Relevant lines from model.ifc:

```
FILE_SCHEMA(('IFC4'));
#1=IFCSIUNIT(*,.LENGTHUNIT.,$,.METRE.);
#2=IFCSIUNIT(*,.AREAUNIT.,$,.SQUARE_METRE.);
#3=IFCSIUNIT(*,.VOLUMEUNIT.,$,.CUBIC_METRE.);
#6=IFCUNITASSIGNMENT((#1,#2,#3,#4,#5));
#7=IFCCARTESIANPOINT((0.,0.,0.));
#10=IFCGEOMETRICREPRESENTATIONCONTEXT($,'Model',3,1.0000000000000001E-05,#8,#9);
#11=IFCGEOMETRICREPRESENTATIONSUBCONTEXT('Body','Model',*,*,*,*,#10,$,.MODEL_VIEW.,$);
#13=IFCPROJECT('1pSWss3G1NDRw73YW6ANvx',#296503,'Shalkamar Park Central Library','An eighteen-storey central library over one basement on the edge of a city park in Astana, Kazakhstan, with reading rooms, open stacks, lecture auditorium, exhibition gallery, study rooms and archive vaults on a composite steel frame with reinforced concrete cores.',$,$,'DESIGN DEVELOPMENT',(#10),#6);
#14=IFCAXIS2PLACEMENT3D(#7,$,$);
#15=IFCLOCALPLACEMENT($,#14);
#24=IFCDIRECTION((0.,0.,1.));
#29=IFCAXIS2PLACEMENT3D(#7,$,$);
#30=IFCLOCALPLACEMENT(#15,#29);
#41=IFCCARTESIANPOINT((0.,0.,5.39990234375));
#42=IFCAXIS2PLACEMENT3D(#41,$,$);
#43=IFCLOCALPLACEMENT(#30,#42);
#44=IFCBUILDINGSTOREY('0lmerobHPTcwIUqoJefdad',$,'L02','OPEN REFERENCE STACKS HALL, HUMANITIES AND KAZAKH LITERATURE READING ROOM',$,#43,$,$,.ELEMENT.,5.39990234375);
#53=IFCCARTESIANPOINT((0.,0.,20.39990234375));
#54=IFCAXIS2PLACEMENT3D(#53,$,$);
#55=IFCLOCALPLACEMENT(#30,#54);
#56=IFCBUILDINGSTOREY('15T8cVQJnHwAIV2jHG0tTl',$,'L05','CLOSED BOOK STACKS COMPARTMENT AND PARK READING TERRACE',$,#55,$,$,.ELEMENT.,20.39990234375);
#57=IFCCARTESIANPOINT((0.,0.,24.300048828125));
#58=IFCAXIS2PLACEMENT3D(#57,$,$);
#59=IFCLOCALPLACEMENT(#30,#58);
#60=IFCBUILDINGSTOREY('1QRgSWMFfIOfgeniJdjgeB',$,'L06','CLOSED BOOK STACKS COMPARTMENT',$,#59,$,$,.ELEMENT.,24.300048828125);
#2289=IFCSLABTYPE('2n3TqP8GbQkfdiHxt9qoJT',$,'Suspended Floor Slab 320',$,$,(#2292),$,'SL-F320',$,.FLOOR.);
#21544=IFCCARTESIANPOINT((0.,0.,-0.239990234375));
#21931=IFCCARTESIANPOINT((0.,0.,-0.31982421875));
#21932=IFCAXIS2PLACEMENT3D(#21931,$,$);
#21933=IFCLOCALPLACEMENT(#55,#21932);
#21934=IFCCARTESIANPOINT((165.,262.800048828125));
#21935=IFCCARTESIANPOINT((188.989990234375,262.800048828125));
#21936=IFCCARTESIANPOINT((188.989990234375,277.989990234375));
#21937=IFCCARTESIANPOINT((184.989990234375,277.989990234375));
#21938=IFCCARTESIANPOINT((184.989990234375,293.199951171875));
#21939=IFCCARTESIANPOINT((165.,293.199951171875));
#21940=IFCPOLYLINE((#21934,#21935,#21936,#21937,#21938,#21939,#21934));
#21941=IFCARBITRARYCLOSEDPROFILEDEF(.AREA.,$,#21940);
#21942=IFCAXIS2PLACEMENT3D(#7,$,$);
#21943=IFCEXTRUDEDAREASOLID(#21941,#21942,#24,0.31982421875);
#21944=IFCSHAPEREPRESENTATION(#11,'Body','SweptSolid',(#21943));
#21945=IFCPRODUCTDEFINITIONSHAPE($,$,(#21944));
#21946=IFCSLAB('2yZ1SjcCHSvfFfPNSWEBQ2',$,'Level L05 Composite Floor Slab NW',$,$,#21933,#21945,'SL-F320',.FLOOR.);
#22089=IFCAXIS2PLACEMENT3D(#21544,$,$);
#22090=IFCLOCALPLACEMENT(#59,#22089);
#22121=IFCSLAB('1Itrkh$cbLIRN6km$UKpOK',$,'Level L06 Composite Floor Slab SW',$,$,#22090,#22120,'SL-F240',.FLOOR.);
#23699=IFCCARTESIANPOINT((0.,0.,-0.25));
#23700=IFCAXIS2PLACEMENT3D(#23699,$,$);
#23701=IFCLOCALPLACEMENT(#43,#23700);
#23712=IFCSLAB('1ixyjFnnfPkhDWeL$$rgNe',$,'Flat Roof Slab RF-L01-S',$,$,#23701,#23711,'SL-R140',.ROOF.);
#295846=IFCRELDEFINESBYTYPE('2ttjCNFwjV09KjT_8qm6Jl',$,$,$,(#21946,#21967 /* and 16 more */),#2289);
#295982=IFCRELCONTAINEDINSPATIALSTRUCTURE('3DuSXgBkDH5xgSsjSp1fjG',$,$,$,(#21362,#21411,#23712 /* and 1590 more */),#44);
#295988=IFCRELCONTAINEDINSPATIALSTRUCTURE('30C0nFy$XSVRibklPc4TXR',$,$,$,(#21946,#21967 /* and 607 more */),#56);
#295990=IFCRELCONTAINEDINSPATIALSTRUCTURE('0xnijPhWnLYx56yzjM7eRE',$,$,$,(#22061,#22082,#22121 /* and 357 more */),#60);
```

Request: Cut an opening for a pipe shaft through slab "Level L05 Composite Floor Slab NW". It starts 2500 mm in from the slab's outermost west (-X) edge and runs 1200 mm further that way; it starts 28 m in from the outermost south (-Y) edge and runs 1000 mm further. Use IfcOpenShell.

```python
import numpy as np
import ifcopenshell
import ifcopenshell.api.feature
import ifcopenshell.api.geometry
import ifcopenshell.api.root
import ifcopenshell.geom
import ifcopenshell.util.placement
import ifcopenshell.util.representation
import ifcopenshell.util.shape
import ifcopenshell.util.unit

model = ifcopenshell.open("model.ifc")
unit_scale = ifcopenshell.util.unit.calculate_unit_scale(model)
settings = ifcopenshell.geom.settings()


def volume(element):
    """Net volume in cubic metres, openings subtracted."""
    shape = ifcopenshell.geom.create_shape(settings, element)
    return ifcopenshell.util.shape.get_volume(shape.geometry)


slab = model.by_guid("2yZ1SjcCHSvfFfPNSWEBQ2")
before = volume(slab)

# Extent in the slab's own axes, in metres. The edges named are its -X and -Y sides.
slab_shape = ifcopenshell.geom.create_shape(settings, slab)
vertices = ifcopenshell.util.shape.get_vertices(slab_shape.geometry)
x_min, y_min, bottom = vertices.min(axis=0)
top = vertices[:, 2].max()

opening = ifcopenshell.api.root.create_entity(model, ifc_class="IfcOpeningElement", name="Pipe shaft opening", predefined_type="OPENING")
context = ifcopenshell.util.representation.get_context(model, "Model", "Body", "MODEL_VIEW")
width, depth = 1.2, 1
outline = [(0.0, 0.0), (width, 0.0), (width, depth), (0.0, depth), (0.0, 0.0)]
# Overshoot both faces by 50 mm so the cut is clean.
shape = ifcopenshell.api.geometry.add_slab_representation(
    model, context=context, depth=top - bottom + 0.1, polyline=outline
)
ifcopenshell.api.geometry.assign_representation(model, product=opening, representation=shape)

matrix = ifcopenshell.util.placement.get_local_placement(slab.ObjectPlacement)
matrix[:, 3] = matrix @ np.append(np.array([x_min + 2.5, y_min + 28, bottom - 0.05]) / unit_scale, 1.0)
ifcopenshell.api.geometry.edit_object_placement(model, product=opening, matrix=matrix, is_si=False)
ifcopenshell.api.feature.add_feature(model, feature=opening, element=slab)

after = volume(slab)

print(f"slab volume {before:.3f} -> {after:.3f} m3")

model.write("model_updated.ifc")
```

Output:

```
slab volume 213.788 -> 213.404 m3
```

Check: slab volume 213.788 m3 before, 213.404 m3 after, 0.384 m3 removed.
